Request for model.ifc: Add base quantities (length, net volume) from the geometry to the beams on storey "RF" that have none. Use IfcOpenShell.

First a look at what the model holds.

```python
import ifcopenshell
import ifcopenshell.util.element
import ifcopenshell.util.unit

model = ifcopenshell.open("model.ifc")
print(model.schema)
for unit_type in ("LENGTHUNIT", "AREAUNIT", "VOLUMEUNIT"):
    print(unit_type, ifcopenshell.util.unit.calculate_unit_scale(model, unit_type))
storey = next(s for s in model.by_type("IfcBuildingStorey") if s.Name == "RF")
beams = [e for e in ifcopenshell.util.element.get_decomposition(storey) if e.is_a("IfcBeam")]
for e in sorted(beams, key=lambda e: e.id()):
    print(e.id(), e.is_a(), e.Name, list(ifcopenshell.util.element.get_psets(e, qtos_only=True)), sep=" | ")
```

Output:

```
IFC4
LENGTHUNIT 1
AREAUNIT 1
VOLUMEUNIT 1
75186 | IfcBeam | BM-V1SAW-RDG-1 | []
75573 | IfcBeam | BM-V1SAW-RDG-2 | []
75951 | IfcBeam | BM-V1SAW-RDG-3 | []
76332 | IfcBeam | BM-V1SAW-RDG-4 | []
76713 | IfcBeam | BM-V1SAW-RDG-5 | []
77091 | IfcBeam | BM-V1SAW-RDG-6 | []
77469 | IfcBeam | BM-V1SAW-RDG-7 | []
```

```python
import ifcopenshell
import ifcopenshell.api.pset
import ifcopenshell.geom
import ifcopenshell.util.element
import ifcopenshell.util.shape
import ifcopenshell.util.unit

model = ifcopenshell.open("model.ifc")
unit_scale = ifcopenshell.util.unit.calculate_unit_scale(model)
volume_scale = ifcopenshell.util.unit.calculate_unit_scale(model, "VOLUMEUNIT")
settings = ifcopenshell.geom.settings()

storey = next(s for s in model.by_type("IfcBuildingStorey") if s.Name == "RF")
beams = [e for e in ifcopenshell.util.element.get_decomposition(storey) if e.is_a("IfcBeam")]

for e in sorted(beams, key=lambda e: e.id()):
    if ifcopenshell.util.element.get_psets(e, qtos_only=True, should_inherit=False):
        continue
    # Geometry comes back in metres, in the element's own axes.
    shape = ifcopenshell.geom.create_shape(settings, e)
    values = {
        "Length": ifcopenshell.util.shape.get_max_xyz(shape.geometry) / unit_scale,
        "NetVolume": ifcopenshell.util.shape.get_volume(shape.geometry) / volume_scale,
    }
    qto = ifcopenshell.api.pset.add_qto(model, product=e, name="Qto_BeamBaseQuantities")
    ifcopenshell.api.pset.edit_qto(model, qto=qto, properties=values)
    print(e.id(), {k: round(v, 3) for k, v in values.items()})

model.write("model_v2.ifc")
```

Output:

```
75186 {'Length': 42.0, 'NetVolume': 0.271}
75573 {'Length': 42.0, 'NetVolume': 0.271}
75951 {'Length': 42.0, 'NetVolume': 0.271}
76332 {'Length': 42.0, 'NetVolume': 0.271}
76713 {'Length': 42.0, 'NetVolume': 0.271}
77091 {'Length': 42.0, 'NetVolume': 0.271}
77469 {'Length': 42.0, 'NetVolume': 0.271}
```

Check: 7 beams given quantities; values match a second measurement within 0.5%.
